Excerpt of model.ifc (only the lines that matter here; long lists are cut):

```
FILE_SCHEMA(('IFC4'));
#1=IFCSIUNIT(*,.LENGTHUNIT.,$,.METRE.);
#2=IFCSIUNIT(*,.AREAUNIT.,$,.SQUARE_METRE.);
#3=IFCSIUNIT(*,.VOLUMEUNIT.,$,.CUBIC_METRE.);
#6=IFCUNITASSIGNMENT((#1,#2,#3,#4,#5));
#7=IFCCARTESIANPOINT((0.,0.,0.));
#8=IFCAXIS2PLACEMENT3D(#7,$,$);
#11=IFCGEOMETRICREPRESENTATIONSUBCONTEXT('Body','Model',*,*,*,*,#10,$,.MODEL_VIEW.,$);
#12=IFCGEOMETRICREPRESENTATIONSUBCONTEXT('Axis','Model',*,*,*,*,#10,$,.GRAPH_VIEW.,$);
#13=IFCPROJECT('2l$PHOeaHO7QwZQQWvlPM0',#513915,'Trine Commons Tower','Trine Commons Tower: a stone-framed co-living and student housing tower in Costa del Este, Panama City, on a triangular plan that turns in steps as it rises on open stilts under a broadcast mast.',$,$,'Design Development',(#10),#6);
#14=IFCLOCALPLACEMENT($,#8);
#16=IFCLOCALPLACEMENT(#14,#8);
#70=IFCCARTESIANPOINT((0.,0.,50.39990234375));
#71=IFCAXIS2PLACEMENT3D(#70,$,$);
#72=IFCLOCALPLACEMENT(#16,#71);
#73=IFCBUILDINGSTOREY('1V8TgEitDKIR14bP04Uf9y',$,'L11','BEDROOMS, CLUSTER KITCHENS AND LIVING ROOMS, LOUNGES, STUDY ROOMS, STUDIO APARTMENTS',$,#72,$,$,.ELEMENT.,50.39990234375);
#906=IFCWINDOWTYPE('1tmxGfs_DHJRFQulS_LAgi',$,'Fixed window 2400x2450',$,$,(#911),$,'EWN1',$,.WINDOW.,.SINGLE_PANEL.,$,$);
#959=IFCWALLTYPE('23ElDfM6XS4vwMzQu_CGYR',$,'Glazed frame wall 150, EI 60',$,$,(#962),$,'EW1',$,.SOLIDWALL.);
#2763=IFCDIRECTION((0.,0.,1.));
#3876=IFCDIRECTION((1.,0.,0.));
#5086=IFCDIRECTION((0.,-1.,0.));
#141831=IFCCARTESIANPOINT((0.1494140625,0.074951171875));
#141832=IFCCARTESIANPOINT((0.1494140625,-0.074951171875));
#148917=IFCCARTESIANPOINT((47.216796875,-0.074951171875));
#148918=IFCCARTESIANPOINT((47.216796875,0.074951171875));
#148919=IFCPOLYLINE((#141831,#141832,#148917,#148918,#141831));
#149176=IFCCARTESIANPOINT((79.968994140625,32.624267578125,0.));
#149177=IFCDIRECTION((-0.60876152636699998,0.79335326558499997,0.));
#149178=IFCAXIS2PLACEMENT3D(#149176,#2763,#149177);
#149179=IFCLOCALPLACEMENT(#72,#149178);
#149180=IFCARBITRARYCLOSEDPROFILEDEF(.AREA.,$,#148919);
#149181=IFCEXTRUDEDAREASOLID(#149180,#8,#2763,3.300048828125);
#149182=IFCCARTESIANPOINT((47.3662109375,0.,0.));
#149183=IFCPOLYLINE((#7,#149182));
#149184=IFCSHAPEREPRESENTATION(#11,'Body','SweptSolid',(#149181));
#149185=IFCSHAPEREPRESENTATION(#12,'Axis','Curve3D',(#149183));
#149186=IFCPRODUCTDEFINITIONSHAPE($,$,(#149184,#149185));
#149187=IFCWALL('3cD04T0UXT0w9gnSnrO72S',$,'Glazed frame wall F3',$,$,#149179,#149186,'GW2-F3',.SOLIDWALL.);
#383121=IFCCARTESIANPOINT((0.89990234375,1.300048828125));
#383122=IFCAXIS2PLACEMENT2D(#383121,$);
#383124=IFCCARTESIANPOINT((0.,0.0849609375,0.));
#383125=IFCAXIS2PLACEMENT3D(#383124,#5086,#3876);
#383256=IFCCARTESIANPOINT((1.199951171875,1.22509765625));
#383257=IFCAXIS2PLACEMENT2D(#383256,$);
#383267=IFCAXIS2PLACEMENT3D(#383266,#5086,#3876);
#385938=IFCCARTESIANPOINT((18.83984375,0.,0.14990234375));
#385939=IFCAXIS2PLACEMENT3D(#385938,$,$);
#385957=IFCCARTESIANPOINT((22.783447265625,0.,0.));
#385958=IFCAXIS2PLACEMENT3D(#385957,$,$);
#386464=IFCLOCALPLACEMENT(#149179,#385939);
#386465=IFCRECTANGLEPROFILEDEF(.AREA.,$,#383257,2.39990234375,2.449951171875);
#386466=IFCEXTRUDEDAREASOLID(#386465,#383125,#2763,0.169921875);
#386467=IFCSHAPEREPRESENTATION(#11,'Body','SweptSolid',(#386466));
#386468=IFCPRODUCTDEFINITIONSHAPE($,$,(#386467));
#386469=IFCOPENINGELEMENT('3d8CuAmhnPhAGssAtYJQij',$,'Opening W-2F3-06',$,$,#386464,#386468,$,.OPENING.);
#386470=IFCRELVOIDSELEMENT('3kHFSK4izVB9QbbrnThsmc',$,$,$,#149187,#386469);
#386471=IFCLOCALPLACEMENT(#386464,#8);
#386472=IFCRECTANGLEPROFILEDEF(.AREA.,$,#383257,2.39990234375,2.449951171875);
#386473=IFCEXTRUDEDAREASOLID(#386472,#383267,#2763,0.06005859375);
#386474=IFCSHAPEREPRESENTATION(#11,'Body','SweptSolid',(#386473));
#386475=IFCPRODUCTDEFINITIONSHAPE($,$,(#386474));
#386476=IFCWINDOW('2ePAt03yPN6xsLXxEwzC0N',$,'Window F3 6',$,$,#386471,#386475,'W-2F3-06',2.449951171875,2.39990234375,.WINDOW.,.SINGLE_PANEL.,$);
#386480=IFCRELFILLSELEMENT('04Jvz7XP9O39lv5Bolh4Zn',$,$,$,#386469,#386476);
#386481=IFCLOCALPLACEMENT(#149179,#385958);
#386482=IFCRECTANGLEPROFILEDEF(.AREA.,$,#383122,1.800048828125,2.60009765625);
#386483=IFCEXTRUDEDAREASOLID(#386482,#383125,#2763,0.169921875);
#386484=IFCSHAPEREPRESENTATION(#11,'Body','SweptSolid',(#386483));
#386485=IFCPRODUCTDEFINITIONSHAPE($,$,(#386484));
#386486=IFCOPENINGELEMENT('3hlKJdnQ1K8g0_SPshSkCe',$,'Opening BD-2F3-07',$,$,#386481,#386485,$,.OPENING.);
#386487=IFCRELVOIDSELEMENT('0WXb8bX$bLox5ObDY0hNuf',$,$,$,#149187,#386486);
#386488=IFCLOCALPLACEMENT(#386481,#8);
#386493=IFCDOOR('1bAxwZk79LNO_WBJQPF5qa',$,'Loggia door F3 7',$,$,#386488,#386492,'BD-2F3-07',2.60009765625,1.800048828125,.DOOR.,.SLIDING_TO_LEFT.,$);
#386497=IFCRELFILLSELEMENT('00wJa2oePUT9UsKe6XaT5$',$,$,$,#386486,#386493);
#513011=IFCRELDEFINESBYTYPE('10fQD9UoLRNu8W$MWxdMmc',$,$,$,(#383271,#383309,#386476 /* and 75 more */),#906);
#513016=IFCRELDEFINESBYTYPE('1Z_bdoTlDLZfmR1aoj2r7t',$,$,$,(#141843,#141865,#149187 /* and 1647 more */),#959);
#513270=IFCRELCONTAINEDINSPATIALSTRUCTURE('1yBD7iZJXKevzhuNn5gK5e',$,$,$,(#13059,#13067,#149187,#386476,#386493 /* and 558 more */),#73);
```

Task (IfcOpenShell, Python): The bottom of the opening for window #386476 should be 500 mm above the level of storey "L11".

```python
import numpy as np
import ifcopenshell
import ifcopenshell.api.geometry
import ifcopenshell.geom
import ifcopenshell.util.element
import ifcopenshell.util.placement
import ifcopenshell.util.shape
import ifcopenshell.util.unit

model = ifcopenshell.open("model.ifc")
unit_scale = ifcopenshell.util.unit.calculate_unit_scale(model)

window = model.by_guid("2ePAt03yPN6xsLXxEwzC0N")
opening = window.FillsVoids[0].RelatingOpeningElement
storey = ifcopenshell.util.element.get_container(window, ifc_class="IfcBuildingStorey")
level = ifcopenshell.util.placement.get_local_placement(storey.ObjectPlacement)[2, 3]

# The opening's origin need not be at the sill, so measure its lowest point.
shape = ifcopenshell.geom.create_shape(ifcopenshell.geom.settings(), opening)
bottom = ifcopenshell.util.shape.get_shape_bottom_elevation(shape, shape.geometry) / unit_scale
dz = level + 0.5 / unit_scale - bottom

shift = np.array([0.0, 0.0, dz])
# The window is placed relative to its opening, so it follows when the opening moves.
matrix = ifcopenshell.util.placement.get_local_placement(opening.ObjectPlacement)
matrix[:3, 3] += shift
ifcopenshell.api.geometry.edit_object_placement(
    model, product=opening, matrix=matrix, is_si=False, should_transform_children=True
)

print(f"moved by {dz * unit_scale:+.3f} m")

model.write("model_v2.ifc")
```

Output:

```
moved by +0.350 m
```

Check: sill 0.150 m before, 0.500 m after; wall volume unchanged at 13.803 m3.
